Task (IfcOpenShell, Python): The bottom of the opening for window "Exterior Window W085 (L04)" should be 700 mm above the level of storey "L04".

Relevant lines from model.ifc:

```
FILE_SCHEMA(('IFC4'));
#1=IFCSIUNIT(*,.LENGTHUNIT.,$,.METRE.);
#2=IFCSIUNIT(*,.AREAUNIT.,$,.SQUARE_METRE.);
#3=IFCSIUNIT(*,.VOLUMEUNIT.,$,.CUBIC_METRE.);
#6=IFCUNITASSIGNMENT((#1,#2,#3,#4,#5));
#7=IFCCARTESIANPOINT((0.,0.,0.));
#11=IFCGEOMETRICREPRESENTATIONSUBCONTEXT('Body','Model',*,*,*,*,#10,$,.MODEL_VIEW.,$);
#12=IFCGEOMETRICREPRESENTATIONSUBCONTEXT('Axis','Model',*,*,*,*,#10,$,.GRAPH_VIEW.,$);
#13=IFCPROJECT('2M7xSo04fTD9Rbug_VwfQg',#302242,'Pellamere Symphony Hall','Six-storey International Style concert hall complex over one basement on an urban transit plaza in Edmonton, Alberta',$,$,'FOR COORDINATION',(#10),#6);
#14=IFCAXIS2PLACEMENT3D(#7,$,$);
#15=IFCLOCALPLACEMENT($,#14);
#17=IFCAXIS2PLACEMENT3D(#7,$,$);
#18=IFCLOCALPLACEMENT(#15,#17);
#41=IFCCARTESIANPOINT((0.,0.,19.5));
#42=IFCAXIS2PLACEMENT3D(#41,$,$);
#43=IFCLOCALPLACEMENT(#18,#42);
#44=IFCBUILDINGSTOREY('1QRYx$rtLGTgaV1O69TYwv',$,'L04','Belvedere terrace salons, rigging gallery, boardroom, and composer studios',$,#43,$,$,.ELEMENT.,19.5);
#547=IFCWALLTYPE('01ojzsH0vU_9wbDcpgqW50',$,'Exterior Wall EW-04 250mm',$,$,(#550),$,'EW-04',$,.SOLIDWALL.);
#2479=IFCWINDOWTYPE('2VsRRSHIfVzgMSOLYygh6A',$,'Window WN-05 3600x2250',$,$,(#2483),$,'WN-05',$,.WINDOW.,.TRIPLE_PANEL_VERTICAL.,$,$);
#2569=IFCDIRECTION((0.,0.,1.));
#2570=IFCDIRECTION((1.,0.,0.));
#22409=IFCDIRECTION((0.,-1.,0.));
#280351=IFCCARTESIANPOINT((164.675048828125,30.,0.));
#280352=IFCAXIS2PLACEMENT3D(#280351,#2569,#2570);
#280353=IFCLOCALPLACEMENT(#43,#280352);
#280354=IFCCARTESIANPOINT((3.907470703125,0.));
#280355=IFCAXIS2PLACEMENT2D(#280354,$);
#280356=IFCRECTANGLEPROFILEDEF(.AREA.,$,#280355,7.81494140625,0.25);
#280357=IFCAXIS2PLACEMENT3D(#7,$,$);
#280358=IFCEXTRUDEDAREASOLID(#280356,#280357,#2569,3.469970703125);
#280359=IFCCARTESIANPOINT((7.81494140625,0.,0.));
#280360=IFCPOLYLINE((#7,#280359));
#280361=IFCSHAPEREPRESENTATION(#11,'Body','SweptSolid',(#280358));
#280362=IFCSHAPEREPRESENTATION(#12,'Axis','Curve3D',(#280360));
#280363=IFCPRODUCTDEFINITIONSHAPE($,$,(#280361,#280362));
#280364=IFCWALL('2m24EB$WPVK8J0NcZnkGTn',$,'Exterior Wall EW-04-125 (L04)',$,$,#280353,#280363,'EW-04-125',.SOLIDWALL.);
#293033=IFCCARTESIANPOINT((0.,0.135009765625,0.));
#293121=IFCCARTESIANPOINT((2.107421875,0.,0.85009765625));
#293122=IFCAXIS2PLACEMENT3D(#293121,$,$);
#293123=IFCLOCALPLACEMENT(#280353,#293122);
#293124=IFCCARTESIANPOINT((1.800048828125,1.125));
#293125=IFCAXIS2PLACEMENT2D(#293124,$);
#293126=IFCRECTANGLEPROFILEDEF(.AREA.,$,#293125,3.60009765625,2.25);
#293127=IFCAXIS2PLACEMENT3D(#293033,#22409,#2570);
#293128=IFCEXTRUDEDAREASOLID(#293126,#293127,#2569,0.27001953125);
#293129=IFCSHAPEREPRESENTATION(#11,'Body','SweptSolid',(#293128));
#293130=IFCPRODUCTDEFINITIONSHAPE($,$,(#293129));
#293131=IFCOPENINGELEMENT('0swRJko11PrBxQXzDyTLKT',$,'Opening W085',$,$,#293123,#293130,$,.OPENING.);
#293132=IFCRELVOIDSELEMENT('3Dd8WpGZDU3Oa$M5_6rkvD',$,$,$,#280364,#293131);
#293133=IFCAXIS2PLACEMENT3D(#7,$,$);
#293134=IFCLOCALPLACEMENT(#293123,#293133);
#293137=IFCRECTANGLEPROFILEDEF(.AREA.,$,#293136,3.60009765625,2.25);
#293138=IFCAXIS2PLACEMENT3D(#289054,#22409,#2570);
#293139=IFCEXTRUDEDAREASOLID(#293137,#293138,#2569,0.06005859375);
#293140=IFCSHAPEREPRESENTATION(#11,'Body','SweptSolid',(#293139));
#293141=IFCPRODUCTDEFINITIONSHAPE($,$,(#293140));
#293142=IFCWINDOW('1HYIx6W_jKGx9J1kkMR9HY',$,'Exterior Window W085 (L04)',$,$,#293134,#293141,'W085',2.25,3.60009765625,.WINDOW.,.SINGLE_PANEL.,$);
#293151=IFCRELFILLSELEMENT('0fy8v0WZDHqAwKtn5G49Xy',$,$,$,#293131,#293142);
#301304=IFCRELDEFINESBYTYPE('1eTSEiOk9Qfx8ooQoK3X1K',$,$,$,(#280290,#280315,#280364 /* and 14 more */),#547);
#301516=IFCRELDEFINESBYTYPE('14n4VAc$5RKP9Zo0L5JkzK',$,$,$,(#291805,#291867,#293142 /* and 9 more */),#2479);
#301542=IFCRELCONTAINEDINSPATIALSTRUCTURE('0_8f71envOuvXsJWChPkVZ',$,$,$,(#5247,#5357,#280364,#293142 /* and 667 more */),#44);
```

```python
import numpy as np
import ifcopenshell
import ifcopenshell.api.geometry
import ifcopenshell.geom
import ifcopenshell.util.element
import ifcopenshell.util.placement
import ifcopenshell.util.shape
import ifcopenshell.util.unit

model = ifcopenshell.open("model.ifc")
unit_scale = ifcopenshell.util.unit.calculate_unit_scale(model)

window = model.by_guid("1HYIx6W_jKGx9J1kkMR9HY")
opening = window.FillsVoids[0].RelatingOpeningElement
storey = ifcopenshell.util.element.get_container(window, ifc_class="IfcBuildingStorey")
level = ifcopenshell.util.placement.get_local_placement(storey.ObjectPlacement)[2, 3]

# The opening's origin need not be at the sill, so measure its lowest point.
shape = ifcopenshell.geom.create_shape(ifcopenshell.geom.settings(), opening)
bottom = ifcopenshell.util.shape.get_shape_bottom_elevation(shape, shape.geometry) / unit_scale
dz = level + 0.7 - bottom

shift = np.array([0.0, 0.0, dz])
# The window is placed relative to its opening, so it follows when the opening moves.
matrix = ifcopenshell.util.placement.get_local_placement(opening.ObjectPlacement)
matrix[:3, 3] += shift
ifcopenshell.api.geometry.edit_object_placement(
    model, product=opening, matrix=matrix, is_si=False, should_transform_children=True
)

print(f"moved by {dz * unit_scale:+.3f} m")

model.write("model_rev.ifc")
```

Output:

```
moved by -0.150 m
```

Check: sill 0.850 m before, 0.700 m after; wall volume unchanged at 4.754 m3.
